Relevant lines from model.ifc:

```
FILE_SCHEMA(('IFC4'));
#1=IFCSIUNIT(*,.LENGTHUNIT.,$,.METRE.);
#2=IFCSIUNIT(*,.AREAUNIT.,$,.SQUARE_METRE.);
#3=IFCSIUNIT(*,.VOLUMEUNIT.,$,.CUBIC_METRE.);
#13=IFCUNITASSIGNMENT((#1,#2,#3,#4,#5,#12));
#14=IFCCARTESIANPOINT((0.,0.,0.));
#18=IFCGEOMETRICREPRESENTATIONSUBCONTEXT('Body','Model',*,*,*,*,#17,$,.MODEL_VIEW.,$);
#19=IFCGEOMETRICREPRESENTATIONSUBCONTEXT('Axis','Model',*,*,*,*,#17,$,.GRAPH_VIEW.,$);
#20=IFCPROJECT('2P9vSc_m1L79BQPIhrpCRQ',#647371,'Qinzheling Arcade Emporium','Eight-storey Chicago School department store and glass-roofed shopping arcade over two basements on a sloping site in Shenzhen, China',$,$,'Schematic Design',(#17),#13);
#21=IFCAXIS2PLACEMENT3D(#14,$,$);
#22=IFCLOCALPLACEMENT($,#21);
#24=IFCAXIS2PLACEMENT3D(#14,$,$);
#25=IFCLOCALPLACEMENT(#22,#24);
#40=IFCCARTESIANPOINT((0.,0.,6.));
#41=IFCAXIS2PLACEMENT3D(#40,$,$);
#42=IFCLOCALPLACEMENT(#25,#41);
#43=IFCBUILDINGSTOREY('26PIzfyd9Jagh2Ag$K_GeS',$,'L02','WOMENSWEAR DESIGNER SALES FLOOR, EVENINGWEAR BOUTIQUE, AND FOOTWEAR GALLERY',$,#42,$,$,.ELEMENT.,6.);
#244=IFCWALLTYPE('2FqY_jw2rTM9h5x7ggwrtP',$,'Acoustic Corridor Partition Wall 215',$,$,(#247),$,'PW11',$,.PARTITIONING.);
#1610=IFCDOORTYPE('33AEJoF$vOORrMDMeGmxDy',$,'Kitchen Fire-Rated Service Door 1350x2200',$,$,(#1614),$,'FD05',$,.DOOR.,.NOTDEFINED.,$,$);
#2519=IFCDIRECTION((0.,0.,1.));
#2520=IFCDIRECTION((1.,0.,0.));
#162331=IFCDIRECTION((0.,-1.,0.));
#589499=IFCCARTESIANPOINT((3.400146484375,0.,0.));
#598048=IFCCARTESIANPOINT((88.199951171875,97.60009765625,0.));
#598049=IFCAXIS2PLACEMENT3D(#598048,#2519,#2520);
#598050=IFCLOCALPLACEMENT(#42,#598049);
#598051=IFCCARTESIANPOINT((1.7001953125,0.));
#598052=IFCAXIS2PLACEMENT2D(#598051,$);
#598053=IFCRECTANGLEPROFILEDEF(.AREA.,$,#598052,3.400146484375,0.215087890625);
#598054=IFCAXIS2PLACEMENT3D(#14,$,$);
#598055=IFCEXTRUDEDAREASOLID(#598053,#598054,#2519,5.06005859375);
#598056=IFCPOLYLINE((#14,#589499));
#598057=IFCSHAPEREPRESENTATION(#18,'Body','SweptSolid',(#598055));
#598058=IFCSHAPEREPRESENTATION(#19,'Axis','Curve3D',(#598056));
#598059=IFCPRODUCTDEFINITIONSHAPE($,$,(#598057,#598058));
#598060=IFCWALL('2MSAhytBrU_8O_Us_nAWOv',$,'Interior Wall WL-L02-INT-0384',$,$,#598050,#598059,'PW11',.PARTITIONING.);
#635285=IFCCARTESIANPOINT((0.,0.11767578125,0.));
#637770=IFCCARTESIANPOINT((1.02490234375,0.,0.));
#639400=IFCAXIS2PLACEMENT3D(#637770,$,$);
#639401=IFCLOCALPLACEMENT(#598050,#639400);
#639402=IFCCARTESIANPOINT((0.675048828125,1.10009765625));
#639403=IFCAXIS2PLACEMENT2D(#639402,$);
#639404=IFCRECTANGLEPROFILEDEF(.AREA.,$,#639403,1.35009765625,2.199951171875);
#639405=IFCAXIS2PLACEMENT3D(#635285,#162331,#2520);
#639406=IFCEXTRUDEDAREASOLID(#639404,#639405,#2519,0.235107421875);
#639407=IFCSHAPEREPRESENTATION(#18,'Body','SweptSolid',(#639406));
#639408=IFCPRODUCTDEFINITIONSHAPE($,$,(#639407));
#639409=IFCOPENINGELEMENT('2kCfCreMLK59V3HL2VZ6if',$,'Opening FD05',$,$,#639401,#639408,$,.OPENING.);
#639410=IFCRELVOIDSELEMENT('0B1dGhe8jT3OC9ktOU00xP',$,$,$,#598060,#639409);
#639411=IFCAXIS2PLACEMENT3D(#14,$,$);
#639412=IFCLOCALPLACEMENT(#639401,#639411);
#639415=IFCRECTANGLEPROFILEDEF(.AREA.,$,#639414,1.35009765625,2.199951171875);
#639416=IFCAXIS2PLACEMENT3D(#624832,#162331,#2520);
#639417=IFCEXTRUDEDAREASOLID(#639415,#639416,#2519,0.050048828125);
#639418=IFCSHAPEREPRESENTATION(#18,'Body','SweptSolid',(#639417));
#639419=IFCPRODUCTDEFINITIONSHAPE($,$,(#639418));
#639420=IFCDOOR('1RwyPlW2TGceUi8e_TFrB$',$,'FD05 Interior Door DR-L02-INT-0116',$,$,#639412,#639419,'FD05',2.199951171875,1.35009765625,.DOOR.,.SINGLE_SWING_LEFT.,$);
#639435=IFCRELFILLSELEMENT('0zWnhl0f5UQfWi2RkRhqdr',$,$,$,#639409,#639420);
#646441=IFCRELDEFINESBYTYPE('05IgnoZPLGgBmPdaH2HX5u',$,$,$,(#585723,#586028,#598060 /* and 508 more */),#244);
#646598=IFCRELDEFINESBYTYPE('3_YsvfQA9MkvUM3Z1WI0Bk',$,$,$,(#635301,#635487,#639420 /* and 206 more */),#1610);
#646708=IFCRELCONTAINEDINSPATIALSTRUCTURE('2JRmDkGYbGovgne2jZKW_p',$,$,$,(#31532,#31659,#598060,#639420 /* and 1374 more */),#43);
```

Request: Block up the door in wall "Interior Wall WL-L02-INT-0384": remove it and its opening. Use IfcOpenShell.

```python
import ifcopenshell
import ifcopenshell.api.feature
import ifcopenshell.api.root
import ifcopenshell.geom
import ifcopenshell.util.shape

model = ifcopenshell.open("model.ifc")
settings = ifcopenshell.geom.settings()


def volume(element):
    """Net volume in cubic metres, openings subtracted."""
    shape = ifcopenshell.geom.create_shape(settings, element)
    return ifcopenshell.util.shape.get_volume(shape.geometry)


door = model.by_guid("1RwyPlW2TGceUi8e_TFrB$")
opening = door.FillsVoids[0].RelatingOpeningElement
wall = opening.VoidsElements[0].RelatingBuildingElement
before = volume(wall)

ifcopenshell.api.root.remove_product(model, product=door)
ifcopenshell.api.feature.remove_feature(model, feature=opening)

after = volume(wall)

print(f"wall volume {before:.3f} -> {after:.3f} m3")

model.write("model-out.ifc")
```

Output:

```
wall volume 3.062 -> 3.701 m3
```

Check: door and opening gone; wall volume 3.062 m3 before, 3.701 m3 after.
